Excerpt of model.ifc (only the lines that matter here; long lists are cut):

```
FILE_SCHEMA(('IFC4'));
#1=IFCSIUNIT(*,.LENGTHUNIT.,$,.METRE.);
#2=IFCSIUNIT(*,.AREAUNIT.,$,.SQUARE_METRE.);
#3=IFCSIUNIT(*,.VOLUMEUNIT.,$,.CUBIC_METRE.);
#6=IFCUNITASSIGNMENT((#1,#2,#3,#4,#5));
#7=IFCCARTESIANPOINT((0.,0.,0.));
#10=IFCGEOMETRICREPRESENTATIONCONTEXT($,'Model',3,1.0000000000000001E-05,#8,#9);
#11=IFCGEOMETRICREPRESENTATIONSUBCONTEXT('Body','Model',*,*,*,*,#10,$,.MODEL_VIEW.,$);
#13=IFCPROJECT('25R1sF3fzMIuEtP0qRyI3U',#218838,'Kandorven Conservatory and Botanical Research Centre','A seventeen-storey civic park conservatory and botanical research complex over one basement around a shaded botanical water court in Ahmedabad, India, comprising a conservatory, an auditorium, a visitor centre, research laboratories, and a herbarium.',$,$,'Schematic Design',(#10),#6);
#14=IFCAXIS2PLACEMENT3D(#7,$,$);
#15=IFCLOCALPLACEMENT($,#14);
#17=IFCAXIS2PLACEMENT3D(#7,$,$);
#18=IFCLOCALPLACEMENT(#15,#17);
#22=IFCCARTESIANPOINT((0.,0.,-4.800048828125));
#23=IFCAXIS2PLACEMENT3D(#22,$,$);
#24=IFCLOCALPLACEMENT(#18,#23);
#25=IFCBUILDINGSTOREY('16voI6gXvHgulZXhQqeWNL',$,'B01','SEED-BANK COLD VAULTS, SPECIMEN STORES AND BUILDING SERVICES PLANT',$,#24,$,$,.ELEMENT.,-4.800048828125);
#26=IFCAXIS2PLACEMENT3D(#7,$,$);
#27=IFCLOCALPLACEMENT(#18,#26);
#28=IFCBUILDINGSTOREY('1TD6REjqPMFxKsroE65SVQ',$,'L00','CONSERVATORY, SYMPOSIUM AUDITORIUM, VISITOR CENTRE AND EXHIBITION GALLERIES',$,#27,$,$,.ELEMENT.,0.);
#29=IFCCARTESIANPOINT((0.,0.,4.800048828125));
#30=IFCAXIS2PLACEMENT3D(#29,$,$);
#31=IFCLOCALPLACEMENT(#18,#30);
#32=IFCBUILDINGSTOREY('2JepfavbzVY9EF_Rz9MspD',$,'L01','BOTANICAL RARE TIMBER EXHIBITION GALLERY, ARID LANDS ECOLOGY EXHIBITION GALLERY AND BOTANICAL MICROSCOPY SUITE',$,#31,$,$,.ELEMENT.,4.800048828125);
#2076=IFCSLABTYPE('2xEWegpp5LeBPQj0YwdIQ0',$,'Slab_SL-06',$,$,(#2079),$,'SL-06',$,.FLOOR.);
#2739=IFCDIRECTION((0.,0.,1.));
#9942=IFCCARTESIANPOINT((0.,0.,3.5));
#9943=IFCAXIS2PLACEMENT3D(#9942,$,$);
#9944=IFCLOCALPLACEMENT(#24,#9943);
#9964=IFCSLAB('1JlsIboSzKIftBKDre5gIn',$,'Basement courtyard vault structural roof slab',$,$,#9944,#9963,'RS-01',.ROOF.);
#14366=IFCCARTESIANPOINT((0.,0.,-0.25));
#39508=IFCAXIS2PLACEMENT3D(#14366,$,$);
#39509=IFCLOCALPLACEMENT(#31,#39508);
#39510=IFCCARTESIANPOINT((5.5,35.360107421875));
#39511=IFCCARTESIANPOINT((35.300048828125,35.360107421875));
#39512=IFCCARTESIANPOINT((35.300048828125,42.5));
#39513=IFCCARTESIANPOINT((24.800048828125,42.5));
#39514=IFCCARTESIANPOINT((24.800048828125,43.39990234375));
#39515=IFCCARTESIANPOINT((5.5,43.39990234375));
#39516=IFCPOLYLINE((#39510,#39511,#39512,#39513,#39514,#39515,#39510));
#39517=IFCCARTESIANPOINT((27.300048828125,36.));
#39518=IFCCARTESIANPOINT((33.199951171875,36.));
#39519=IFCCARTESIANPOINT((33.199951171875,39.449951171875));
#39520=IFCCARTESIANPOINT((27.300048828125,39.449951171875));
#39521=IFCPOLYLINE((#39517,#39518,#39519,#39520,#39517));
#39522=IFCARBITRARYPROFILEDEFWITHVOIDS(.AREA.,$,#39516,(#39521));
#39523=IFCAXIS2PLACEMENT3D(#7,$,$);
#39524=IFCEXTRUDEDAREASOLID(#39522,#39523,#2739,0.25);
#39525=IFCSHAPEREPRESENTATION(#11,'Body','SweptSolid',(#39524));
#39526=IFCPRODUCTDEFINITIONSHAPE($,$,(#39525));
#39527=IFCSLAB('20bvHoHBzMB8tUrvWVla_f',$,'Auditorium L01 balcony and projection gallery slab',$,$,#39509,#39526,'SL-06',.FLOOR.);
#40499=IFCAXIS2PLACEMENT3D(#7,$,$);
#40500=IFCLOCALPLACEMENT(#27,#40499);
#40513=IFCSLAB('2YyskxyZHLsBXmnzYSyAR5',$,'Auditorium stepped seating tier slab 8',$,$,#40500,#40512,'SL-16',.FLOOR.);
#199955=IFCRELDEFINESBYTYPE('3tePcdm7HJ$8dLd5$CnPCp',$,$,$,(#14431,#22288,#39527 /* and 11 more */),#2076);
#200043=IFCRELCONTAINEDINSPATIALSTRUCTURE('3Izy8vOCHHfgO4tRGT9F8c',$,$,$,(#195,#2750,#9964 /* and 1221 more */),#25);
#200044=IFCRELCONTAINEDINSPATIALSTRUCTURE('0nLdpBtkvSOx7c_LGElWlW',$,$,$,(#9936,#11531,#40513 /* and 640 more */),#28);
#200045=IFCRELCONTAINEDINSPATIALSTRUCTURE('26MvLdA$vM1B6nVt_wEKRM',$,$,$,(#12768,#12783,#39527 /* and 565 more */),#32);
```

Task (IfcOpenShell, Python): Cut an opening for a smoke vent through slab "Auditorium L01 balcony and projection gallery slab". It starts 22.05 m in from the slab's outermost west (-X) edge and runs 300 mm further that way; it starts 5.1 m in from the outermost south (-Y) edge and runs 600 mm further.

```python
import numpy as np
import ifcopenshell
import ifcopenshell.api.feature
import ifcopenshell.api.geometry
import ifcopenshell.api.root
import ifcopenshell.geom
import ifcopenshell.util.placement
import ifcopenshell.util.representation
import ifcopenshell.util.shape
import ifcopenshell.util.unit

model = ifcopenshell.open("model.ifc")
unit_scale = ifcopenshell.util.unit.calculate_unit_scale(model)
settings = ifcopenshell.geom.settings()


def volume(element):
    """Net volume in cubic metres, openings subtracted."""
    shape = ifcopenshell.geom.create_shape(settings, element)
    return ifcopenshell.util.shape.get_volume(shape.geometry)


slab = model.by_id(39527)
before = volume(slab)

# Extent in the slab's own axes, in metres. The edges named are its -X and -Y sides.
slab_shape = ifcopenshell.geom.create_shape(settings, slab)
vertices = ifcopenshell.util.shape.get_vertices(slab_shape.geometry)
x_min, y_min, bottom = vertices.min(axis=0)
top = vertices[:, 2].max()

opening = ifcopenshell.api.root.create_entity(model, ifc_class="IfcOpeningElement", name="Smoke vent opening", predefined_type="OPENING")
context = ifcopenshell.util.representation.get_context(model, "Model", "Body", "MODEL_VIEW")
width, depth = 0.3, 0.6
outline = [(0.0, 0.0), (width, 0.0), (width, depth), (0.0, depth), (0.0, 0.0)]
# Overshoot both faces by 50 mm so the cut is clean.
shape = ifcopenshell.api.geometry.add_slab_representation(
    model, context=context, depth=top - bottom + 0.1, polyline=outline
)
ifcopenshell.api.geometry.assign_representation(model, product=opening, representation=shape)

matrix = ifcopenshell.util.placement.get_local_placement(slab.ObjectPlacement)
matrix[:, 3] = matrix @ np.append(np.array([x_min + 22.05, y_min + 5.1, bottom - 0.05]) / unit_scale, 1.0)
ifcopenshell.api.geometry.edit_object_placement(model, product=opening, matrix=matrix, is_si=False)
ifcopenshell.api.feature.add_feature(model, feature=opening, element=slab)

after = volume(slab)

print(f"slab volume {before:.3f} -> {after:.3f} m3")

model.write("model_edited.ifc")
```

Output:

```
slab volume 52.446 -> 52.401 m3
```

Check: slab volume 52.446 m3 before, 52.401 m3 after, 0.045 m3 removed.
